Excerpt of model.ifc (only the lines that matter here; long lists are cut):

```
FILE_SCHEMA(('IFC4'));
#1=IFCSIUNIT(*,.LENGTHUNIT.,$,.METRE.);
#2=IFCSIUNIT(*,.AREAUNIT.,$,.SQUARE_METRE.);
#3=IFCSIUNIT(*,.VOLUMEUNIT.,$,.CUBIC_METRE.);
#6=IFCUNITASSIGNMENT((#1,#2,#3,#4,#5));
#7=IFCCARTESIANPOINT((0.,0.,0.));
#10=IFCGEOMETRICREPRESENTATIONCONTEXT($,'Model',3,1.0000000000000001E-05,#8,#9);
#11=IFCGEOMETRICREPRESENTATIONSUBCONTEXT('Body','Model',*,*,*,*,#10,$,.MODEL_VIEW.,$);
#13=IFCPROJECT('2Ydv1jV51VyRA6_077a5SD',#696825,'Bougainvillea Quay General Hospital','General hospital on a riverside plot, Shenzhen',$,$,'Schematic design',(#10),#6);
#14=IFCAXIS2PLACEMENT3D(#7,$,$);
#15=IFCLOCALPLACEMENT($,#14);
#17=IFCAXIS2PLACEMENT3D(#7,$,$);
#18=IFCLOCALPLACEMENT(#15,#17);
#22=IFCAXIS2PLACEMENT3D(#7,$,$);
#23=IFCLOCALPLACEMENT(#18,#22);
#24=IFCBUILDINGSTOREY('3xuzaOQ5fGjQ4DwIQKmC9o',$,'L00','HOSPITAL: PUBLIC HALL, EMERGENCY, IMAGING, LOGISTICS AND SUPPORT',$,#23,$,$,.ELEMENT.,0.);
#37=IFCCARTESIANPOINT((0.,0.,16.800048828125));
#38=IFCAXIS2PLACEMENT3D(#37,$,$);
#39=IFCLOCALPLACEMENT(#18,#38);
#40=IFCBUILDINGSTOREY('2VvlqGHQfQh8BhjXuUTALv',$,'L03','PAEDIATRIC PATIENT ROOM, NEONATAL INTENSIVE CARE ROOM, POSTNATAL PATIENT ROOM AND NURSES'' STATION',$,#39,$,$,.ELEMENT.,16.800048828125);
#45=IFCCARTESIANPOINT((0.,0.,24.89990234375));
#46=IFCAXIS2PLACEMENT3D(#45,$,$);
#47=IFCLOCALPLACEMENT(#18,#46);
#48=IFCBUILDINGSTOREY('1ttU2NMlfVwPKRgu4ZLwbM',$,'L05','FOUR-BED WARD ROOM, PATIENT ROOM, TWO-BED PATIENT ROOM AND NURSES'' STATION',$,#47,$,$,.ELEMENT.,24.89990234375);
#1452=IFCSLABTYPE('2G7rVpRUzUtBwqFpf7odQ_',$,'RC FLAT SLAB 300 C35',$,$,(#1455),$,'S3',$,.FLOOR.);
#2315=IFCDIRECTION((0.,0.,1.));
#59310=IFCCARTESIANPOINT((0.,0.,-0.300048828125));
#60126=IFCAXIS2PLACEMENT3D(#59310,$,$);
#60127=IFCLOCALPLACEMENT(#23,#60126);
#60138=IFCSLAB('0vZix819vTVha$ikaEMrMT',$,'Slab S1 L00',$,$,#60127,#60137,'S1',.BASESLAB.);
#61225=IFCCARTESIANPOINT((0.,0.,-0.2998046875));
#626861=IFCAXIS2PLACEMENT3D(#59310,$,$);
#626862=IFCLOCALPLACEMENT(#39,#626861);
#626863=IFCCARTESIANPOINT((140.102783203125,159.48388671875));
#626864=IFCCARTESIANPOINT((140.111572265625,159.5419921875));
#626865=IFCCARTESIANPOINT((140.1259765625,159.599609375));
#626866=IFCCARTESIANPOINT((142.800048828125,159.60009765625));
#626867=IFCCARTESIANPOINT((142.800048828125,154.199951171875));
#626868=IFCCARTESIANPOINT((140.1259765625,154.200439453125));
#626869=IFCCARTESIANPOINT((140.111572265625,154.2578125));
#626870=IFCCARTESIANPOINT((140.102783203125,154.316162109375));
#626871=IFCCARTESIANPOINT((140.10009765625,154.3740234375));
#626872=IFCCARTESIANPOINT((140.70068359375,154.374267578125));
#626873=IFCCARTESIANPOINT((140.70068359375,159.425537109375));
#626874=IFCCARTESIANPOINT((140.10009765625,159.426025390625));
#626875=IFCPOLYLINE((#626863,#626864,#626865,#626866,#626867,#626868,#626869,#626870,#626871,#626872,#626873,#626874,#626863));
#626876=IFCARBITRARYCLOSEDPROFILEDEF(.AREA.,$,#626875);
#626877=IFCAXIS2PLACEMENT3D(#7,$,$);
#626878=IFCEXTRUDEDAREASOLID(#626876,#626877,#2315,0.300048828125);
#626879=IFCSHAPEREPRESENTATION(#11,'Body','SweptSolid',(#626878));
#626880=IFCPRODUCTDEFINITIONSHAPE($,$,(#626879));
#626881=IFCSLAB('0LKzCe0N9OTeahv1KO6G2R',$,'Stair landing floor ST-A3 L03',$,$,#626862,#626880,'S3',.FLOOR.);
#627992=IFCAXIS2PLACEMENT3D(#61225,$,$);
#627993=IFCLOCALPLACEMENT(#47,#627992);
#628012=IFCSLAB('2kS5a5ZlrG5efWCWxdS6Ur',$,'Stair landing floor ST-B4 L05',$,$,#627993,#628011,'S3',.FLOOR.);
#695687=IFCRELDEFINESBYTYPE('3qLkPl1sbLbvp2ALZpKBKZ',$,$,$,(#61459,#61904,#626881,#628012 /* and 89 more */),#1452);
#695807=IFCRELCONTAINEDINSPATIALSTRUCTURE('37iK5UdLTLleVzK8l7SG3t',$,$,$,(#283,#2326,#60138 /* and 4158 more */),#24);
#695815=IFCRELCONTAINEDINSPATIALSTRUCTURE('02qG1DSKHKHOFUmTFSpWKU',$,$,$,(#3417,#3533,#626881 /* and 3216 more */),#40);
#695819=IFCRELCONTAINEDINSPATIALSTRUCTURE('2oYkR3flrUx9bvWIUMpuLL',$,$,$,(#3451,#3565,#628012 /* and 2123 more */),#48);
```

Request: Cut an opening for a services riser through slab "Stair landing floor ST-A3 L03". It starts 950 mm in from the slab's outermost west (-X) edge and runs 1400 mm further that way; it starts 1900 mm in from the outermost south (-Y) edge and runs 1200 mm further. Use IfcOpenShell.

```python
import numpy as np
import ifcopenshell
import ifcopenshell.api.feature
import ifcopenshell.api.geometry
import ifcopenshell.api.root
import ifcopenshell.geom
import ifcopenshell.util.placement
import ifcopenshell.util.representation
import ifcopenshell.util.shape
import ifcopenshell.util.unit

model = ifcopenshell.open("model.ifc")
unit_scale = ifcopenshell.util.unit.calculate_unit_scale(model)
settings = ifcopenshell.geom.settings()


def volume(element):
    """Net volume in cubic metres, openings subtracted."""
    shape = ifcopenshell.geom.create_shape(settings, element)
    return ifcopenshell.util.shape.get_volume(shape.geometry)


slab = model.by_id(626881)
before = volume(slab)

# Extent in the slab's own axes, in metres. The edges named are its -X and -Y sides.
slab_shape = ifcopenshell.geom.create_shape(settings, slab)
vertices = ifcopenshell.util.shape.get_vertices(slab_shape.geometry)
x_min, y_min, bottom = vertices.min(axis=0)
top = vertices[:, 2].max()

opening = ifcopenshell.api.root.create_entity(model, ifc_class="IfcOpeningElement", name="Services riser opening", predefined_type="OPENING")
context = ifcopenshell.util.representation.get_context(model, "Model", "Body", "MODEL_VIEW")
width, depth = 1.4, 1.2
outline = [(0.0, 0.0), (width, 0.0), (width, depth), (0.0, depth), (0.0, 0.0)]
# Overshoot both faces by 50 mm so the cut is clean.
shape = ifcopenshell.api.geometry.add_slab_representation(
    model, context=context, depth=top - bottom + 0.1, polyline=outline
)
ifcopenshell.api.geometry.assign_representation(model, product=opening, representation=shape)

matrix = ifcopenshell.util.placement.get_local_placement(slab.ObjectPlacement)
matrix[:, 3] = matrix @ np.append(np.array([x_min + 0.95, y_min + 1.9, bottom - 0.05]) / unit_scale, 1.0)
ifcopenshell.api.geometry.edit_object_placement(model, product=opening, matrix=matrix, is_si=False)
ifcopenshell.api.feature.add_feature(model, feature=opening, element=slab)

after = volume(slab)

print(f"slab volume {before:.3f} -> {after:.3f} m3")

model.write("model-out.ifc")
```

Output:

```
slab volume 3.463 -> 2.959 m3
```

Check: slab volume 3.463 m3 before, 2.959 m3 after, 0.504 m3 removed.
